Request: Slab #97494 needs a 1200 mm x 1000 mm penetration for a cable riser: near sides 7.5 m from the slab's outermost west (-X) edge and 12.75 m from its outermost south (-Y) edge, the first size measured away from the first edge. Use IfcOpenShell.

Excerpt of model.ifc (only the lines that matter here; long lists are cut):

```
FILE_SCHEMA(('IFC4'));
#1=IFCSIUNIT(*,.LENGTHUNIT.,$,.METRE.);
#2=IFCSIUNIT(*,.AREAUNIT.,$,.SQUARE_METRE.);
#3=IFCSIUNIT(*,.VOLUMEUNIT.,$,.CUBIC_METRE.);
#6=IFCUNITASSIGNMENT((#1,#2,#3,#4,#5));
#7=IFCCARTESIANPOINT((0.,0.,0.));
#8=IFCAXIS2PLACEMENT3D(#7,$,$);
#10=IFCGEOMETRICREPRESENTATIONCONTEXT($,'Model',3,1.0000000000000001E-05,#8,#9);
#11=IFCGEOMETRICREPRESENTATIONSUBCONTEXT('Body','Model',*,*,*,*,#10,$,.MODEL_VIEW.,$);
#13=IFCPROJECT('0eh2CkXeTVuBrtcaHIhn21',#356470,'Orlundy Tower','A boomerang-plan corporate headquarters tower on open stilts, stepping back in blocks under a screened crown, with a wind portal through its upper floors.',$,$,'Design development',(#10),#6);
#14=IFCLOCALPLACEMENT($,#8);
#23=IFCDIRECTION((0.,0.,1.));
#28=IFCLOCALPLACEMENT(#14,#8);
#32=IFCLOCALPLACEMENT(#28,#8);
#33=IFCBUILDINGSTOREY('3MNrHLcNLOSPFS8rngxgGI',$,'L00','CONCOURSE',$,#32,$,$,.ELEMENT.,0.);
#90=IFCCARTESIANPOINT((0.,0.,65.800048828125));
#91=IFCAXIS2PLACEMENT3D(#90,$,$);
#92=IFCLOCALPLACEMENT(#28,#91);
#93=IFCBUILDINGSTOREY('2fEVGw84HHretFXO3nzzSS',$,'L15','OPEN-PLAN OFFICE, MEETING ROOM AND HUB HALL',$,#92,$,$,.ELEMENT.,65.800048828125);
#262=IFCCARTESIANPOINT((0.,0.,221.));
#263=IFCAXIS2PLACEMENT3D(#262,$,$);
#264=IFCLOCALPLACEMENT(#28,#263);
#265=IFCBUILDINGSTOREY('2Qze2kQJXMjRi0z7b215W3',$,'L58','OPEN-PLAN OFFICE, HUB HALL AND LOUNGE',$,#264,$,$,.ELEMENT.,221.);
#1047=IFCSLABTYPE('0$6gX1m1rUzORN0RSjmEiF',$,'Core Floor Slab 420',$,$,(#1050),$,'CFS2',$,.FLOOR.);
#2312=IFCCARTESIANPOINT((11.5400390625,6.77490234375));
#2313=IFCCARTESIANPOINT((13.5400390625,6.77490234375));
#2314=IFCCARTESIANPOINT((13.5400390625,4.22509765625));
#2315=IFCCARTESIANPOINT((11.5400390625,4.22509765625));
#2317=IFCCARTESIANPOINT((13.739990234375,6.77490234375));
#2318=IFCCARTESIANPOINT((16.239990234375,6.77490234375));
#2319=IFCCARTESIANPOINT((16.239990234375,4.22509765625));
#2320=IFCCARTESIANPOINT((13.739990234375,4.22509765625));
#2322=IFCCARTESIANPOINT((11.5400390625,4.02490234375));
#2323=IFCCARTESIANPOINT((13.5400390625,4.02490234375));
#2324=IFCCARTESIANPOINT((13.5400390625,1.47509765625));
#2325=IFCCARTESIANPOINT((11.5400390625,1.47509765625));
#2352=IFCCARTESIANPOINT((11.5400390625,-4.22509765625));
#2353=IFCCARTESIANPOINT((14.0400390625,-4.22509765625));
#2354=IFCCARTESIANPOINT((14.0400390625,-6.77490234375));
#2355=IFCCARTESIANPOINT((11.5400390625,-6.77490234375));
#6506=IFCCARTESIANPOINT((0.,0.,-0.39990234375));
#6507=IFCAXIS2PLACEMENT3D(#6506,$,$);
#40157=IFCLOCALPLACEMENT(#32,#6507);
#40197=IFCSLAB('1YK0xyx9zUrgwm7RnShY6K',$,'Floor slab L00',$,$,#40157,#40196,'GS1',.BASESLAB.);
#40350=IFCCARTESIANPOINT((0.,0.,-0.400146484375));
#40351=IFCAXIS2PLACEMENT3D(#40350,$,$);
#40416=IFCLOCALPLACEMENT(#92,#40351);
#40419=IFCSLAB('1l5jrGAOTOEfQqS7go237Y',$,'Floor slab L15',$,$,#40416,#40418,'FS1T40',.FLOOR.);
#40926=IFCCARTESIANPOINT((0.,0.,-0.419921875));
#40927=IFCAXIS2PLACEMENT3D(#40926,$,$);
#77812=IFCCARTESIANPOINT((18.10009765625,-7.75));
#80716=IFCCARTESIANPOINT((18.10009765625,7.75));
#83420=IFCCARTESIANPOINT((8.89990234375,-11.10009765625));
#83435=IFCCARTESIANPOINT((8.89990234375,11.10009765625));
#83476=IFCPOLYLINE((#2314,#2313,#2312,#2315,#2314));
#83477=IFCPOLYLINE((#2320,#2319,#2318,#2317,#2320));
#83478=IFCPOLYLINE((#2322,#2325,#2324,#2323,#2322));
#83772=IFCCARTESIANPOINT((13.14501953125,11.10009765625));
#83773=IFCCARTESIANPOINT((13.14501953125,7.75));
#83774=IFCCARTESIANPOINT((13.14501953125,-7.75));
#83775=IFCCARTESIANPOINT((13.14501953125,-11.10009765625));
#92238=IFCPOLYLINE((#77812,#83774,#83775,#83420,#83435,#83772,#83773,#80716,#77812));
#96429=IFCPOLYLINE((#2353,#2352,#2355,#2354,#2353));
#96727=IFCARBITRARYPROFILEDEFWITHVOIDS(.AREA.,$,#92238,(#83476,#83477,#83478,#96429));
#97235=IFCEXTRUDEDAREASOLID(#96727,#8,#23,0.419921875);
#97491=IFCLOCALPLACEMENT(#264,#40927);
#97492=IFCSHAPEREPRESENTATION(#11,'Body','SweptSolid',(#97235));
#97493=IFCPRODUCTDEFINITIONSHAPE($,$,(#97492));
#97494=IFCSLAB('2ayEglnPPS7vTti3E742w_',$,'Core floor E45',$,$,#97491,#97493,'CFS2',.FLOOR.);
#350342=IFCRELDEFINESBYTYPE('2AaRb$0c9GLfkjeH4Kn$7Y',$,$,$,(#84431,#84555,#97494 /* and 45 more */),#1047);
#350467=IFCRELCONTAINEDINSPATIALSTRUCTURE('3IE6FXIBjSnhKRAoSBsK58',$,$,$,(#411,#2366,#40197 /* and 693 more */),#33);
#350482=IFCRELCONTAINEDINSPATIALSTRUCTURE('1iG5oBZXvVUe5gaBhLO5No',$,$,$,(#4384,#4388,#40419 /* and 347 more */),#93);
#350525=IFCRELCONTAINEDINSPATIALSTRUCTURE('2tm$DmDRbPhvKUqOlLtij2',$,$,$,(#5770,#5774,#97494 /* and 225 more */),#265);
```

```python
import numpy as np
import ifcopenshell
import ifcopenshell.api.feature
import ifcopenshell.api.geometry
import ifcopenshell.api.root
import ifcopenshell.geom
import ifcopenshell.util.placement
import ifcopenshell.util.representation
import ifcopenshell.util.shape
import ifcopenshell.util.unit

model = ifcopenshell.open("model.ifc")
unit_scale = ifcopenshell.util.unit.calculate_unit_scale(model)
settings = ifcopenshell.geom.settings()


def volume(element):
    """Net volume in cubic metres, openings subtracted."""
    shape = ifcopenshell.geom.create_shape(settings, element)
    return ifcopenshell.util.shape.get_volume(shape.geometry)


slab = model.by_guid("2ayEglnPPS7vTti3E742w_")
before = volume(slab)

# Extent in the slab's own axes, in metres. The edges named are its -X and -Y sides.
slab_shape = ifcopenshell.geom.create_shape(settings, slab)
vertices = ifcopenshell.util.shape.get_vertices(slab_shape.geometry)
x_min, y_min, bottom = vertices.min(axis=0)
top = vertices[:, 2].max()

opening = ifcopenshell.api.root.create_entity(model, ifc_class="IfcOpeningElement", name="Cable riser opening", predefined_type="OPENING")
context = ifcopenshell.util.representation.get_context(model, "Model", "Body", "MODEL_VIEW")
width, depth = 1.2, 1
outline = [(0.0, 0.0), (width, 0.0), (width, depth), (0.0, depth), (0.0, 0.0)]
# Overshoot both faces by 50 mm so the cut is clean.
shape = ifcopenshell.api.geometry.add_slab_representation(
    model, context=context, depth=top - bottom + 0.1, polyline=outline
)
ifcopenshell.api.geometry.assign_representation(model, product=opening, representation=shape)

matrix = ifcopenshell.util.placement.get_local_placement(slab.ObjectPlacement)
matrix[:, 3] = matrix @ np.append(np.array([x_min + 7.5, y_min + 12.75, bottom - 0.05]) / unit_scale, 1.0)
ifcopenshell.api.geometry.edit_object_placement(model, product=opening, matrix=matrix, is_si=False)
ifcopenshell.api.feature.add_feature(model, feature=opening, element=slab)

after = volume(slab)

print(f"slab volume {before:.3f} -> {after:.3f} m3")

model.write("model_rev.ifc")
```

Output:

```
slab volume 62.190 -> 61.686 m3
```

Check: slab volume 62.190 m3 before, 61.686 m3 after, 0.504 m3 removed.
